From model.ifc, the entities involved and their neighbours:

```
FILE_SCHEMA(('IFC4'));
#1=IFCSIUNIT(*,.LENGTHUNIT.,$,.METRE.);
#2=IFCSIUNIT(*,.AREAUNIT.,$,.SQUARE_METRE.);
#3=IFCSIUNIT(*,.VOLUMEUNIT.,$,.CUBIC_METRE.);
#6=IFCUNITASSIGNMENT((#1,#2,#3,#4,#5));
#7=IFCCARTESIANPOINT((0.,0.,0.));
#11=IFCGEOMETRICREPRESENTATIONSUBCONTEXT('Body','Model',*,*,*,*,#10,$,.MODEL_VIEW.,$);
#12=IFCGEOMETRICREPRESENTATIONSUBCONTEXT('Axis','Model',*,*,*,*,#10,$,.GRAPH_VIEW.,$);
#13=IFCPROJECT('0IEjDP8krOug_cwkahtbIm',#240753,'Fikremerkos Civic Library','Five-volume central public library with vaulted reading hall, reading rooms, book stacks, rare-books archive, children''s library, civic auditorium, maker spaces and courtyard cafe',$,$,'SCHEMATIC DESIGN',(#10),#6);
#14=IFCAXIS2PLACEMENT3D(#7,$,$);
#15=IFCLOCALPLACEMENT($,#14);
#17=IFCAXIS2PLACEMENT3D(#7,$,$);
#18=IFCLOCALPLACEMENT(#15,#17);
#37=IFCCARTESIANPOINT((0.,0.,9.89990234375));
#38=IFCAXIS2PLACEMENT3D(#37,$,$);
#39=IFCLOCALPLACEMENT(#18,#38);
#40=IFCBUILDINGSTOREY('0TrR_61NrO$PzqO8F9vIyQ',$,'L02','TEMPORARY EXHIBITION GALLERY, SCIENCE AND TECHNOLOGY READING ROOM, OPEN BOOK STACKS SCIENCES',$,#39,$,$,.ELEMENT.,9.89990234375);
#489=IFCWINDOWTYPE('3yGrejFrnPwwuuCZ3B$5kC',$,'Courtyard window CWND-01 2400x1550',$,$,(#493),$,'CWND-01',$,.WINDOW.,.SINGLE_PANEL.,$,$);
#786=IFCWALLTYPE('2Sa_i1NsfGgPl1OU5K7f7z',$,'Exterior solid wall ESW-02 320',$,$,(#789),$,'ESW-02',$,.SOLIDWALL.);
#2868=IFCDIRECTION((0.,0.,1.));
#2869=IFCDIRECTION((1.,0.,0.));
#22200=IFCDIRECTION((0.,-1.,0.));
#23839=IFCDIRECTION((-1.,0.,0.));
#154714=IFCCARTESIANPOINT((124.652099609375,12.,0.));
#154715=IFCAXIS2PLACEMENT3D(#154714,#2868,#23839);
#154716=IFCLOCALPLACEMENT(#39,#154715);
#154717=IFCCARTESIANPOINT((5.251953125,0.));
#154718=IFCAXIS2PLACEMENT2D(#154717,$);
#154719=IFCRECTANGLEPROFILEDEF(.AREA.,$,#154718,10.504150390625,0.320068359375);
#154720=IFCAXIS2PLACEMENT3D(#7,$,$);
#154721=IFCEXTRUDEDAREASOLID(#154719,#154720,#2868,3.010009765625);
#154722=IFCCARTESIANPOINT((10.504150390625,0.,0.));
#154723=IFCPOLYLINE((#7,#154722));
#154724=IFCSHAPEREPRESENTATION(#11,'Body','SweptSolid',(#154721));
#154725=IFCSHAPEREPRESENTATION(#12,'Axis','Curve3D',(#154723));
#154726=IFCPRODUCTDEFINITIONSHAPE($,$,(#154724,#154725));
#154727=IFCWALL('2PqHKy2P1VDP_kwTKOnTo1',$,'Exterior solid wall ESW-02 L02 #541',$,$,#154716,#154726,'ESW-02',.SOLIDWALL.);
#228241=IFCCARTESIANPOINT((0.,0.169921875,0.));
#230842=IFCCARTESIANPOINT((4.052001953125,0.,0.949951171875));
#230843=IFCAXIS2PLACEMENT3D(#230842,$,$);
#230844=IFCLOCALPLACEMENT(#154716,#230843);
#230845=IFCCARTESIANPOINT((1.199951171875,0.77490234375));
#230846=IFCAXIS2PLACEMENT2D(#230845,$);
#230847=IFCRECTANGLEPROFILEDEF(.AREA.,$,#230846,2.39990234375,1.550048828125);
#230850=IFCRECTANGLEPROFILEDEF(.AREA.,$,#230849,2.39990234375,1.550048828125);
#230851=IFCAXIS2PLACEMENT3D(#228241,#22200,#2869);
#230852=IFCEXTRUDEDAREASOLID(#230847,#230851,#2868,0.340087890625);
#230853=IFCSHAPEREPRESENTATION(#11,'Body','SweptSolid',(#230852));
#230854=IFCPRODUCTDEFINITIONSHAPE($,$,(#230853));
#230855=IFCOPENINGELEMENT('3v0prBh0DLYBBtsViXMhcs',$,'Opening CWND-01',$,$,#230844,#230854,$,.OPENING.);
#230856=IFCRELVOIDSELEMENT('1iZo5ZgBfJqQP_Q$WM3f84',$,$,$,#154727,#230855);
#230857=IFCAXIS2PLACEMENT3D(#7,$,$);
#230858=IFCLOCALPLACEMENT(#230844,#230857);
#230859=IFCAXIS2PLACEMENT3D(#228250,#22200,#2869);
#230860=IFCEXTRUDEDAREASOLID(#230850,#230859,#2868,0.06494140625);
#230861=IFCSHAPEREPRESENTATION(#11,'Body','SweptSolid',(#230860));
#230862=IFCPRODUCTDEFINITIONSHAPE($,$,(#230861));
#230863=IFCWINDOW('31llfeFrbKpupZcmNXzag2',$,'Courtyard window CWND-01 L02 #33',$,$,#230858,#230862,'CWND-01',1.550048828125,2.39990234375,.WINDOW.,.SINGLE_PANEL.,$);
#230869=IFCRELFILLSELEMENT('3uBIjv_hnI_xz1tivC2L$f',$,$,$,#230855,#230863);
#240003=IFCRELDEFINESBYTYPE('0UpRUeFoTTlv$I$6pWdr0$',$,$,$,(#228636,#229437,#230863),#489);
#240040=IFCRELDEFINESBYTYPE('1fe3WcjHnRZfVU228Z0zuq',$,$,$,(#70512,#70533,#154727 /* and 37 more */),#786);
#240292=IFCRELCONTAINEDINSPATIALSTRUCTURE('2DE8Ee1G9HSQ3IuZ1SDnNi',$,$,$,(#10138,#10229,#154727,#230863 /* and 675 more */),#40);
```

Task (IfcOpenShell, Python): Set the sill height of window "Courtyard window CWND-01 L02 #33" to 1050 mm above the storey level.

```python
import numpy as np
import ifcopenshell
import ifcopenshell.api.geometry
import ifcopenshell.geom
import ifcopenshell.util.element
import ifcopenshell.util.placement
import ifcopenshell.util.shape
import ifcopenshell.util.unit

model = ifcopenshell.open("model.ifc")
unit_scale = ifcopenshell.util.unit.calculate_unit_scale(model)

window = model.by_guid("31llfeFrbKpupZcmNXzag2")
opening = window.FillsVoids[0].RelatingOpeningElement
storey = ifcopenshell.util.element.get_container(window, ifc_class="IfcBuildingStorey")
level = ifcopenshell.util.placement.get_local_placement(storey.ObjectPlacement)[2, 3]

# The opening's origin need not be at the sill, so measure its lowest point.
shape = ifcopenshell.geom.create_shape(ifcopenshell.geom.settings(), opening)
bottom = ifcopenshell.util.shape.get_shape_bottom_elevation(shape, shape.geometry) / unit_scale
dz = level + 1.05 / unit_scale - bottom

shift = np.array([0.0, 0.0, dz])
# The window is placed relative to its opening, so it follows when the opening moves.
matrix = ifcopenshell.util.placement.get_local_placement(opening.ObjectPlacement)
matrix[:3, 3] += shift
ifcopenshell.api.geometry.edit_object_placement(
    model, product=opening, matrix=matrix, is_si=False, should_transform_children=True
)

print(f"moved by {dz * unit_scale:+.3f} m")

model.write("model_v2.ifc")
```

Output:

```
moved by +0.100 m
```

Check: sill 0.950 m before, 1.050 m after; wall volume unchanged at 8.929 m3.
